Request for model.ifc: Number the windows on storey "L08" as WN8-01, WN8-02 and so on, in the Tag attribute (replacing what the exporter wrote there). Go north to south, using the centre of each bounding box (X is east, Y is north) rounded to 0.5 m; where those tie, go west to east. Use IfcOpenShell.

First a look at what the model holds.

```python
import ifcopenshell
import ifcopenshell.util.element
import ifcopenshell.util.placement

model = ifcopenshell.open("model.ifc")
print(model.schema)
storey = next(s for s in model.by_type("IfcBuildingStorey") if s.Name == "L08")
windows = [e for e in ifcopenshell.util.element.get_decomposition(storey) if e.is_a("IfcWindow")]
for e in sorted(windows, key=lambda e: e.id()):
    origin = ifcopenshell.util.placement.get_local_placement(e.ObjectPlacement)[:3, 3]
    print(e.id(), e.Tag, e.Name, origin.round(2) + 0.0, sep=" | ")
```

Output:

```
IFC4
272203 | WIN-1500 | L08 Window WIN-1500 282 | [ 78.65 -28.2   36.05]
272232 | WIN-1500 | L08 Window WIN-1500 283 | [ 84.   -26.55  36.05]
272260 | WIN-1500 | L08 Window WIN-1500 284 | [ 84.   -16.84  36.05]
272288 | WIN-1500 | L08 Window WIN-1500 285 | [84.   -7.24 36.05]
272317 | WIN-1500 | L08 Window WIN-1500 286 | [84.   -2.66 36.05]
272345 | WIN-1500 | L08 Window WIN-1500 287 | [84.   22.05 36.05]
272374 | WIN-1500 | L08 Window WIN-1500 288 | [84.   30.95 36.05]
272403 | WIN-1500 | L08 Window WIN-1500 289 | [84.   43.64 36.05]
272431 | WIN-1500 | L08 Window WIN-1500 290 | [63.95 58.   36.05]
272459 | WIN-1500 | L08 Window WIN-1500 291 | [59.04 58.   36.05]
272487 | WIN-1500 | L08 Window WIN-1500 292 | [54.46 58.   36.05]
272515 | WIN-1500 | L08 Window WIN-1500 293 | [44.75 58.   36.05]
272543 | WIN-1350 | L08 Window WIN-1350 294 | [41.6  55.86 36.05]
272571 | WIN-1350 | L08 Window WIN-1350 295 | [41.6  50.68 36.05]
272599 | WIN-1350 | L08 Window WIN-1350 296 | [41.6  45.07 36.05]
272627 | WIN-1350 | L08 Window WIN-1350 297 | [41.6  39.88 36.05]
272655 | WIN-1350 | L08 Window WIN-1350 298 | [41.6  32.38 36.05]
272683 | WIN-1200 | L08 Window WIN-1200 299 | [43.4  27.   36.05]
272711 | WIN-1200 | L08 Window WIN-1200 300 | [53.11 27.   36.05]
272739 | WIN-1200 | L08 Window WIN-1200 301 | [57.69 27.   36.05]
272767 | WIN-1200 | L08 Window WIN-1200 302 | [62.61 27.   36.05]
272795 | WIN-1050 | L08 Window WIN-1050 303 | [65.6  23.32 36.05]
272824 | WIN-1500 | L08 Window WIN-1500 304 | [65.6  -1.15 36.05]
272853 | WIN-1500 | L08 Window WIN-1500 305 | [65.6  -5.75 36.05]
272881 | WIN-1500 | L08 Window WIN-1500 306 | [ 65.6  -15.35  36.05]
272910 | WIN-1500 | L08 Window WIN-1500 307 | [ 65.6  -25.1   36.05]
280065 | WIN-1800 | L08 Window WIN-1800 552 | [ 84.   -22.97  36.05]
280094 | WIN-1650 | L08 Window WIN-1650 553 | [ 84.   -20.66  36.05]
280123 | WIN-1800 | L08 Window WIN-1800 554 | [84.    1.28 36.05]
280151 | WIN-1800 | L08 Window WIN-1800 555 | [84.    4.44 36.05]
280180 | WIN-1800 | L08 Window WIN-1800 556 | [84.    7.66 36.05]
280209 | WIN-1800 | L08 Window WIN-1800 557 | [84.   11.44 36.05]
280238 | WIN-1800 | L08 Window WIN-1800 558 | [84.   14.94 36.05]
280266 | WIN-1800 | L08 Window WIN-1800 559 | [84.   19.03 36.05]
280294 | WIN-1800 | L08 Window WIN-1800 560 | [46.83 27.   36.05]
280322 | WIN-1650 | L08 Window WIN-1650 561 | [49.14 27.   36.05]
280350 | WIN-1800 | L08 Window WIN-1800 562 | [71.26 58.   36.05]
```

```python
import ifcopenshell
import ifcopenshell.geom
import ifcopenshell.util.element
import ifcopenshell.util.shape

model = ifcopenshell.open("model.ifc")
settings = ifcopenshell.geom.settings()
settings.set("use-world-coords", True)


def centre(element):
    shape = ifcopenshell.geom.create_shape(settings, element)
    return ifcopenshell.util.shape.get_bbox_centroid(shape.geometry)


storey = next(s for s in model.by_type("IfcBuildingStorey") if s.Name == "L08")
windows = [e for e in ifcopenshell.util.element.get_decomposition(storey) if e.is_a("IfcWindow")]

# Insertion points can sit at a corner or the storey origin, so sort by the geometry (in metres).
centres = {e: centre(e) for e in windows}
windows.sort(key=lambda e: (-round(centres[e][1] / 0.5), centres[e][0]))

for i, e in enumerate(windows, start=1):
    number = f"WN8-{i:02d}"
    e.Tag = number
    print(e.id(), number)

model.write("model_updated.ifc")
```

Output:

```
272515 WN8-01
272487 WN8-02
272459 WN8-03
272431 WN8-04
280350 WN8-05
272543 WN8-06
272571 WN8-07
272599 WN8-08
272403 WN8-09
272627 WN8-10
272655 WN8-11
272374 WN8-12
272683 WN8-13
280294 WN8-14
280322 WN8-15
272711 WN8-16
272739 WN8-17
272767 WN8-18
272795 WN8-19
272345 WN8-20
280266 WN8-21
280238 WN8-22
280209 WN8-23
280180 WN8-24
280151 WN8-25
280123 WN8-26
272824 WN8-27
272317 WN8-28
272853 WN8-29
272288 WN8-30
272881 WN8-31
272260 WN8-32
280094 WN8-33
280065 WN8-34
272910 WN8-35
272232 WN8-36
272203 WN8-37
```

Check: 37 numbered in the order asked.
